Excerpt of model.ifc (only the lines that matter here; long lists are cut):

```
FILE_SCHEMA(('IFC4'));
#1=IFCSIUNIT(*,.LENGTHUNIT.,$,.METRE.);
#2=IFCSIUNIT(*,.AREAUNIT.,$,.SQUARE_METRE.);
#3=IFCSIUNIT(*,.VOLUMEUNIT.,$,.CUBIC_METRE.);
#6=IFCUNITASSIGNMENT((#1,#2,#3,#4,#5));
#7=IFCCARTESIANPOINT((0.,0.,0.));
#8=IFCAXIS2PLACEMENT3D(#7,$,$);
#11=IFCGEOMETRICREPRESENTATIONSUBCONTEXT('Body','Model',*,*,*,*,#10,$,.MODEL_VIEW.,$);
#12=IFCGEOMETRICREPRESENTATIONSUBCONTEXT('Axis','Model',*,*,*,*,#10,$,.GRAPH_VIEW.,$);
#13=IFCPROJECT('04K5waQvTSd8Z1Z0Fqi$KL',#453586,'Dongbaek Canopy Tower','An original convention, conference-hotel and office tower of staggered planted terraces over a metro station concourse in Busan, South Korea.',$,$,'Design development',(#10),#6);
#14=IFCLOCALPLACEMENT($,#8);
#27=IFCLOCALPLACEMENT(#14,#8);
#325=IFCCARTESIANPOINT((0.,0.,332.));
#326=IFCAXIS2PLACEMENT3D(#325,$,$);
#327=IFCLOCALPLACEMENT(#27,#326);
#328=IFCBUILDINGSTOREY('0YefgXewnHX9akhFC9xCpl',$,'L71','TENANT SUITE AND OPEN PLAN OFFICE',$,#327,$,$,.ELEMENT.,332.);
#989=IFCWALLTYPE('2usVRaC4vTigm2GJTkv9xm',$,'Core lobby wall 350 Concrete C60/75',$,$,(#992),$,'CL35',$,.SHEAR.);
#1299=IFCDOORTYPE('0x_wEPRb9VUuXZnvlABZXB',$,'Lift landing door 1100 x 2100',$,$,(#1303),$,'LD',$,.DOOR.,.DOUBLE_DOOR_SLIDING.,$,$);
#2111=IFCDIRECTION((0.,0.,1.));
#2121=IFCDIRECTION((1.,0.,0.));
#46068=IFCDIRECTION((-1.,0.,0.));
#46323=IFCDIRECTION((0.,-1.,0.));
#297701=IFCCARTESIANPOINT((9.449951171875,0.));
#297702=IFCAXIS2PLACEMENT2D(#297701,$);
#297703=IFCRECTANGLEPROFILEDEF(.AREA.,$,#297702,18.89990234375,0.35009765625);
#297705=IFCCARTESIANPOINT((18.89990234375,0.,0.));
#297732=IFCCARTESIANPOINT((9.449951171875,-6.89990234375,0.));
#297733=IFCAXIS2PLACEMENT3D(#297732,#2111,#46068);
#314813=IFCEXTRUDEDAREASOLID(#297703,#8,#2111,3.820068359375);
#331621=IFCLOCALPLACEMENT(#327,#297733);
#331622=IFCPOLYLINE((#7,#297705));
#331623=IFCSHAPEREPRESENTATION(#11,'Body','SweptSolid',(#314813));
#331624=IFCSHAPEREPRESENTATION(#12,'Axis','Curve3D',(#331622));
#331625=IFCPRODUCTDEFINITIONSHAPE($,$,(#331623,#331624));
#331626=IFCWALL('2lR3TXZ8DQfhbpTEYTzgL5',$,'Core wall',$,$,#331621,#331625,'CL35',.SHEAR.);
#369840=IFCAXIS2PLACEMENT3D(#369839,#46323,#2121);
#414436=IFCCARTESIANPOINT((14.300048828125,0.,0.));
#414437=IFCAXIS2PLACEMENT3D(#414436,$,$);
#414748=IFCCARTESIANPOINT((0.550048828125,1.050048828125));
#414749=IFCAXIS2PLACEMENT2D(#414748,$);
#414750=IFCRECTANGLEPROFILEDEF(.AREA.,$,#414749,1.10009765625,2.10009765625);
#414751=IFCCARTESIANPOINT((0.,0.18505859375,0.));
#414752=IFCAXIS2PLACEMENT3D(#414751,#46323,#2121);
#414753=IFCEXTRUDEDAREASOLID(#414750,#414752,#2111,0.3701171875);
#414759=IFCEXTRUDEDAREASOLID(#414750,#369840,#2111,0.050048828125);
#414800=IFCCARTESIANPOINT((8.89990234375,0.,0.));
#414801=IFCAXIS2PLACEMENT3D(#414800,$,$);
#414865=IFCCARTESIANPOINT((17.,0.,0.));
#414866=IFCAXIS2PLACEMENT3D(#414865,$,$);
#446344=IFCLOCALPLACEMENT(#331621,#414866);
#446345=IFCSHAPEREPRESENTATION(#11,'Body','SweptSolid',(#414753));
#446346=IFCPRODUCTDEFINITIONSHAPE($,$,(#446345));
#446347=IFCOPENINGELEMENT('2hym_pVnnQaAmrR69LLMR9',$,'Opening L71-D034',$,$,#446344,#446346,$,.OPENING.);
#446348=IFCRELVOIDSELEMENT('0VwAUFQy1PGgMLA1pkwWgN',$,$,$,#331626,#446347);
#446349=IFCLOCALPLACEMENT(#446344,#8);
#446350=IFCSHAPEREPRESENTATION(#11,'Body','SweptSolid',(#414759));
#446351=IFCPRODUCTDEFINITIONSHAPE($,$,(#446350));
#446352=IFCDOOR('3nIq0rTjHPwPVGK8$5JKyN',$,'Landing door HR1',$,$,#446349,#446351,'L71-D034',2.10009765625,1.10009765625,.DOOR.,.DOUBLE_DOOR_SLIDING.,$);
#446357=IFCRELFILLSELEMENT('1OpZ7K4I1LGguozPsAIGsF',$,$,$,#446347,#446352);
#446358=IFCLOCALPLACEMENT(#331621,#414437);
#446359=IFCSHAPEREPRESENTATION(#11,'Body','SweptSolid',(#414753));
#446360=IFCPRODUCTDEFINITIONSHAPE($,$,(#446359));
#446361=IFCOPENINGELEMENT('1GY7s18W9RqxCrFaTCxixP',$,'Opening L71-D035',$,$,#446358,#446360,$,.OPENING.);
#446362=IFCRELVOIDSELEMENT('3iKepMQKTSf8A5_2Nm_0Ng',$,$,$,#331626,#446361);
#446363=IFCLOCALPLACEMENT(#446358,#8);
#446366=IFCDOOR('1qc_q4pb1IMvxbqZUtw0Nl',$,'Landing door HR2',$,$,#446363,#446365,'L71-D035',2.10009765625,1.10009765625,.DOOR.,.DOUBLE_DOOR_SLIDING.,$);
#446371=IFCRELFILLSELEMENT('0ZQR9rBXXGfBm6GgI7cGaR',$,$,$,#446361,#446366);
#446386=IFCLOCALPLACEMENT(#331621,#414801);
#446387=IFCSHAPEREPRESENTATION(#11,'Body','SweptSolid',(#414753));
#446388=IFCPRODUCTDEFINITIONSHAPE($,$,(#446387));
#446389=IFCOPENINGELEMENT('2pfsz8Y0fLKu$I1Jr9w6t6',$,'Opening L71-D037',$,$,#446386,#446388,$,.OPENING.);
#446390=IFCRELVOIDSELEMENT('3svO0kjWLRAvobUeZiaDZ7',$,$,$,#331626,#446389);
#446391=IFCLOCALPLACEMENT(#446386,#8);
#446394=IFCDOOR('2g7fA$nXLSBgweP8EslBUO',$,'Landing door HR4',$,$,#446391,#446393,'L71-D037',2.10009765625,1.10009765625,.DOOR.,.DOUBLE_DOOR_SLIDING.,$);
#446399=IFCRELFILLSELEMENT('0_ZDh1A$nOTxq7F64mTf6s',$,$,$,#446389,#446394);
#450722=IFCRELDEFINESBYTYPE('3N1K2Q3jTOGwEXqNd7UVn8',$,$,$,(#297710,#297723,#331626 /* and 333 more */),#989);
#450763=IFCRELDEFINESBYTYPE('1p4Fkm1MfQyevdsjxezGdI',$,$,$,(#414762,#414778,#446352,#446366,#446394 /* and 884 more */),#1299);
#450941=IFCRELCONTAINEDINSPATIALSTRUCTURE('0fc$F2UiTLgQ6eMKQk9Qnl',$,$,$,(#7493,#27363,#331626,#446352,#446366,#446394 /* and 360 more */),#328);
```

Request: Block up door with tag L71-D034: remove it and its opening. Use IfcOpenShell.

```python
import ifcopenshell
import ifcopenshell.api.feature
import ifcopenshell.api.root
import ifcopenshell.geom
import ifcopenshell.util.shape

model = ifcopenshell.open("model.ifc")
settings = ifcopenshell.geom.settings()


def volume(element):
    """Net volume in cubic metres, openings subtracted."""
    shape = ifcopenshell.geom.create_shape(settings, element)
    return ifcopenshell.util.shape.get_volume(shape.geometry)


door = model.by_id(446352)
opening = door.FillsVoids[0].RelatingOpeningElement
wall = opening.VoidsElements[0].RelatingBuildingElement
before = volume(wall)

ifcopenshell.api.root.remove_product(model, product=door)
ifcopenshell.api.feature.remove_feature(model, feature=opening)

after = volume(wall)

print(f"wall volume {before:.3f} -> {after:.3f} m3")

model.write("model_rev.ifc")
```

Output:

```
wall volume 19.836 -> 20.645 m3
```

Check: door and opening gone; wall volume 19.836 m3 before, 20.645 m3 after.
